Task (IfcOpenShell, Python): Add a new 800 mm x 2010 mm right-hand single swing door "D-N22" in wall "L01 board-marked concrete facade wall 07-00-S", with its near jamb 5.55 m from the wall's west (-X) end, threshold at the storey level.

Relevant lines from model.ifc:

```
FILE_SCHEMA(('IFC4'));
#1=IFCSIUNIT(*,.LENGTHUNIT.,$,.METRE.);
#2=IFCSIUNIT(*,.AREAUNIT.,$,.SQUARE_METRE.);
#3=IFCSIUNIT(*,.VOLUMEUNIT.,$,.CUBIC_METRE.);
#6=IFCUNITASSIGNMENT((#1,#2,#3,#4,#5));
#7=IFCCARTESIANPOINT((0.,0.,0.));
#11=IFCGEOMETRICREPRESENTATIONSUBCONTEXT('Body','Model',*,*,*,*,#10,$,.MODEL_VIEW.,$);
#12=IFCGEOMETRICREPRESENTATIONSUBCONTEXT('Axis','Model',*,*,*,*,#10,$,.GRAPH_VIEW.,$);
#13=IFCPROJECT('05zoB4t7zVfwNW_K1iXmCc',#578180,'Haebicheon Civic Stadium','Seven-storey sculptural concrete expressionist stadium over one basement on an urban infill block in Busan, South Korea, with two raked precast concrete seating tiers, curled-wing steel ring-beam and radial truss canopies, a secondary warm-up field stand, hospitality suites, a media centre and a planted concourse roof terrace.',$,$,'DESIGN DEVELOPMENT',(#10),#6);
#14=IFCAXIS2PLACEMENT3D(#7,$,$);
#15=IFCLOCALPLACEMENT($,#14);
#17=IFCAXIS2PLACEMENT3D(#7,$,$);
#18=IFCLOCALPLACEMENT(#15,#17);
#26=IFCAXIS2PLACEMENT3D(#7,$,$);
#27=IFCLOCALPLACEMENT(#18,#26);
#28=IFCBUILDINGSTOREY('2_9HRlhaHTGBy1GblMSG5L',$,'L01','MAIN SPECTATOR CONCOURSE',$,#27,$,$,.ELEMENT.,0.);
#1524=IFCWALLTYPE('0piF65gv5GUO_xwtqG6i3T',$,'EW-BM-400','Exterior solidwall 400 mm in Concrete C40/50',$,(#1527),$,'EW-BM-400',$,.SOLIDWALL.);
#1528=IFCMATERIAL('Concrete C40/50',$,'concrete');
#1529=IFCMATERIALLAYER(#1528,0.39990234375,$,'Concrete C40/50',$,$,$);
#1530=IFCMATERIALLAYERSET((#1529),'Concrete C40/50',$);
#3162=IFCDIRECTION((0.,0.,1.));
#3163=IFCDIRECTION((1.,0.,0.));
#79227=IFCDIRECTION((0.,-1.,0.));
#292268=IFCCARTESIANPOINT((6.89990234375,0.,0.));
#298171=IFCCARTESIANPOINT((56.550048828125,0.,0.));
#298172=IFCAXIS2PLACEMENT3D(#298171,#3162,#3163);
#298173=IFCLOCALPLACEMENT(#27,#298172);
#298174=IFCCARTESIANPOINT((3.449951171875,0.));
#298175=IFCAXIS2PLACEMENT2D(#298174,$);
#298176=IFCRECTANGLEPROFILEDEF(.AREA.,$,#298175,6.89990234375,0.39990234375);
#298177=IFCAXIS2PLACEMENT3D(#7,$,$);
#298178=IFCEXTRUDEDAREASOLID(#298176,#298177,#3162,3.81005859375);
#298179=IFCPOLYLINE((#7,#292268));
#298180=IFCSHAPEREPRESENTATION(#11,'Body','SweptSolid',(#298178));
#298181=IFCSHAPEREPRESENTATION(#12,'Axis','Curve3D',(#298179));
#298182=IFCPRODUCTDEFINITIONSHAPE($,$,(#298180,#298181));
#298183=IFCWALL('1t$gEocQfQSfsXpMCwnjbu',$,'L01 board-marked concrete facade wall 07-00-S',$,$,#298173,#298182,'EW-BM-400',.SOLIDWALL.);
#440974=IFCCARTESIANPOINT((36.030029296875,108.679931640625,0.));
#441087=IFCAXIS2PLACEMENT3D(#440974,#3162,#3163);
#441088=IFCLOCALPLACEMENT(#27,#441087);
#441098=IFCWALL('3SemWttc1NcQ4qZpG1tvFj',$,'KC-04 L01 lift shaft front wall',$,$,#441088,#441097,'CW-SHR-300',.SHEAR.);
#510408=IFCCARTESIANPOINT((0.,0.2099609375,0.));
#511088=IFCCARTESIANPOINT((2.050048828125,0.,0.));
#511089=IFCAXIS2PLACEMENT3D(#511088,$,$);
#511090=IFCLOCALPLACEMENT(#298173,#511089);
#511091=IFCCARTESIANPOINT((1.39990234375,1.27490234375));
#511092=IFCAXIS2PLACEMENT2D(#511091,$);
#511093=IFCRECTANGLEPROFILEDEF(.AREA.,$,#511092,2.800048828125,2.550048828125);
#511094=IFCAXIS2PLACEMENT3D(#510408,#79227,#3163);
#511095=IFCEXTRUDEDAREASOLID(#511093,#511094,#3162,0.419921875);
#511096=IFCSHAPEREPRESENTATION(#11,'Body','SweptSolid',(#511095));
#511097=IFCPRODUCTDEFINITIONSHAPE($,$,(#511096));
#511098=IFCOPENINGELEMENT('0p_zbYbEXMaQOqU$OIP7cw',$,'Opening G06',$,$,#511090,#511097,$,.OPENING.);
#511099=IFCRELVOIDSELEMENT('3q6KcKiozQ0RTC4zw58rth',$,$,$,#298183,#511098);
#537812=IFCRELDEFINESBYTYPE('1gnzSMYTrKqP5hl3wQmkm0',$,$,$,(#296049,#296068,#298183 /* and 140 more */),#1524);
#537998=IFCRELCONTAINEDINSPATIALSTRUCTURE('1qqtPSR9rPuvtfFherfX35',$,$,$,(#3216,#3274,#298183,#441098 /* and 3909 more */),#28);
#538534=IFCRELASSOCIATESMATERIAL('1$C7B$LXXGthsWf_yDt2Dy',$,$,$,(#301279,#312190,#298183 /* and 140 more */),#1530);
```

```python
import numpy as np
import ifcopenshell
import ifcopenshell.api.feature
import ifcopenshell.api.geometry
import ifcopenshell.api.root
import ifcopenshell.api.spatial
import ifcopenshell.geom
import ifcopenshell.util.element
import ifcopenshell.util.placement
import ifcopenshell.util.representation
import ifcopenshell.util.shape
import ifcopenshell.util.unit

model = ifcopenshell.open("model.ifc")
unit_scale = ifcopenshell.util.unit.calculate_unit_scale(model)
settings = ifcopenshell.geom.settings()


def volume(element):
    """Net volume in cubic metres, openings subtracted."""
    shape = ifcopenshell.geom.create_shape(settings, element)
    return ifcopenshell.util.shape.get_volume(shape.geometry)


wall = model.by_guid("1t$gEocQfQSfsXpMCwnjbu")
storey = ifcopenshell.util.element.get_container(wall, ifc_class="IfcBuildingStorey")
context = ifcopenshell.util.representation.get_context(model, "Model", "Body", "MODEL_VIEW")
before = volume(wall)

width, height, from_end, sill = 0.8, 2.01, 5.55, 0.0  # metres

# The wall runs along its own X axis, and the end named is its -X end.
wall_shape = ifcopenshell.geom.create_shape(settings, wall)
x, y, z = ifcopenshell.util.shape.get_vertices(wall_shape.geometry).T
start = x.min() + from_end
face, thickness = float(y.min()), float(y.max() - y.min())
wall_matrix = ifcopenshell.util.placement.get_local_placement(wall.ObjectPlacement)
level = ifcopenshell.util.placement.get_local_placement(storey.ObjectPlacement)[2, 3]


def in_wall(x, y):
    """Placement at x, y metres in the wall's axes, at sill height."""
    matrix = wall_matrix.copy()
    matrix[:, 3] = wall_matrix @ np.array([x / unit_scale, y / unit_scale, 0.0, 1.0])
    matrix[2, 3] = level + sill / unit_scale
    return matrix


# Opening: a box that overshoots both wall faces by 50 mm.
opening = ifcopenshell.api.root.create_entity(model, ifc_class="IfcOpeningElement", predefined_type="OPENING")
box = ifcopenshell.api.geometry.add_wall_representation(
    model, context=context, length=width, height=height, thickness=thickness + 0.1
)
ifcopenshell.api.geometry.assign_representation(model, product=opening, representation=box)
ifcopenshell.api.geometry.edit_object_placement(model, product=opening, matrix=in_wall(start, face - 0.05), is_si=False)
ifcopenshell.api.feature.add_feature(model, feature=opening, element=wall)

door = ifcopenshell.api.root.create_entity(model, ifc_class="IfcDoor", name="D-N22", predefined_type="DOOR")
door.OverallWidth, door.OverallHeight = width / unit_scale, height / unit_scale
door.OperationType = "SINGLE_SWING_RIGHT"
body = ifcopenshell.api.geometry.add_door_representation(
    model,
    context=context,
    overall_width=door.OverallWidth,
    overall_height=door.OverallHeight,
    operation_type="SINGLE_SWING_RIGHT",
    lining_properties={"LiningDepth": thickness / unit_scale, "ThresholdDepth": thickness / unit_scale},
)
ifcopenshell.api.geometry.assign_representation(model, product=door, representation=body)
ifcopenshell.api.spatial.assign_container(model, products=[door], relating_structure=storey)
ifcopenshell.api.feature.add_filling(model, opening=opening, element=door)

# The lining spans the wall, so the door starts at the wall face.
ifcopenshell.api.geometry.edit_object_placement(model, product=door, matrix=in_wall(start, face), is_si=False)

after = volume(wall)

print(f"wall volume {before:.3f} -> {after:.3f} m3")

model.write("model_rev.ifc")
```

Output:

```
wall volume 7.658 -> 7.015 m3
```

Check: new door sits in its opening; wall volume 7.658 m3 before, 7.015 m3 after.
